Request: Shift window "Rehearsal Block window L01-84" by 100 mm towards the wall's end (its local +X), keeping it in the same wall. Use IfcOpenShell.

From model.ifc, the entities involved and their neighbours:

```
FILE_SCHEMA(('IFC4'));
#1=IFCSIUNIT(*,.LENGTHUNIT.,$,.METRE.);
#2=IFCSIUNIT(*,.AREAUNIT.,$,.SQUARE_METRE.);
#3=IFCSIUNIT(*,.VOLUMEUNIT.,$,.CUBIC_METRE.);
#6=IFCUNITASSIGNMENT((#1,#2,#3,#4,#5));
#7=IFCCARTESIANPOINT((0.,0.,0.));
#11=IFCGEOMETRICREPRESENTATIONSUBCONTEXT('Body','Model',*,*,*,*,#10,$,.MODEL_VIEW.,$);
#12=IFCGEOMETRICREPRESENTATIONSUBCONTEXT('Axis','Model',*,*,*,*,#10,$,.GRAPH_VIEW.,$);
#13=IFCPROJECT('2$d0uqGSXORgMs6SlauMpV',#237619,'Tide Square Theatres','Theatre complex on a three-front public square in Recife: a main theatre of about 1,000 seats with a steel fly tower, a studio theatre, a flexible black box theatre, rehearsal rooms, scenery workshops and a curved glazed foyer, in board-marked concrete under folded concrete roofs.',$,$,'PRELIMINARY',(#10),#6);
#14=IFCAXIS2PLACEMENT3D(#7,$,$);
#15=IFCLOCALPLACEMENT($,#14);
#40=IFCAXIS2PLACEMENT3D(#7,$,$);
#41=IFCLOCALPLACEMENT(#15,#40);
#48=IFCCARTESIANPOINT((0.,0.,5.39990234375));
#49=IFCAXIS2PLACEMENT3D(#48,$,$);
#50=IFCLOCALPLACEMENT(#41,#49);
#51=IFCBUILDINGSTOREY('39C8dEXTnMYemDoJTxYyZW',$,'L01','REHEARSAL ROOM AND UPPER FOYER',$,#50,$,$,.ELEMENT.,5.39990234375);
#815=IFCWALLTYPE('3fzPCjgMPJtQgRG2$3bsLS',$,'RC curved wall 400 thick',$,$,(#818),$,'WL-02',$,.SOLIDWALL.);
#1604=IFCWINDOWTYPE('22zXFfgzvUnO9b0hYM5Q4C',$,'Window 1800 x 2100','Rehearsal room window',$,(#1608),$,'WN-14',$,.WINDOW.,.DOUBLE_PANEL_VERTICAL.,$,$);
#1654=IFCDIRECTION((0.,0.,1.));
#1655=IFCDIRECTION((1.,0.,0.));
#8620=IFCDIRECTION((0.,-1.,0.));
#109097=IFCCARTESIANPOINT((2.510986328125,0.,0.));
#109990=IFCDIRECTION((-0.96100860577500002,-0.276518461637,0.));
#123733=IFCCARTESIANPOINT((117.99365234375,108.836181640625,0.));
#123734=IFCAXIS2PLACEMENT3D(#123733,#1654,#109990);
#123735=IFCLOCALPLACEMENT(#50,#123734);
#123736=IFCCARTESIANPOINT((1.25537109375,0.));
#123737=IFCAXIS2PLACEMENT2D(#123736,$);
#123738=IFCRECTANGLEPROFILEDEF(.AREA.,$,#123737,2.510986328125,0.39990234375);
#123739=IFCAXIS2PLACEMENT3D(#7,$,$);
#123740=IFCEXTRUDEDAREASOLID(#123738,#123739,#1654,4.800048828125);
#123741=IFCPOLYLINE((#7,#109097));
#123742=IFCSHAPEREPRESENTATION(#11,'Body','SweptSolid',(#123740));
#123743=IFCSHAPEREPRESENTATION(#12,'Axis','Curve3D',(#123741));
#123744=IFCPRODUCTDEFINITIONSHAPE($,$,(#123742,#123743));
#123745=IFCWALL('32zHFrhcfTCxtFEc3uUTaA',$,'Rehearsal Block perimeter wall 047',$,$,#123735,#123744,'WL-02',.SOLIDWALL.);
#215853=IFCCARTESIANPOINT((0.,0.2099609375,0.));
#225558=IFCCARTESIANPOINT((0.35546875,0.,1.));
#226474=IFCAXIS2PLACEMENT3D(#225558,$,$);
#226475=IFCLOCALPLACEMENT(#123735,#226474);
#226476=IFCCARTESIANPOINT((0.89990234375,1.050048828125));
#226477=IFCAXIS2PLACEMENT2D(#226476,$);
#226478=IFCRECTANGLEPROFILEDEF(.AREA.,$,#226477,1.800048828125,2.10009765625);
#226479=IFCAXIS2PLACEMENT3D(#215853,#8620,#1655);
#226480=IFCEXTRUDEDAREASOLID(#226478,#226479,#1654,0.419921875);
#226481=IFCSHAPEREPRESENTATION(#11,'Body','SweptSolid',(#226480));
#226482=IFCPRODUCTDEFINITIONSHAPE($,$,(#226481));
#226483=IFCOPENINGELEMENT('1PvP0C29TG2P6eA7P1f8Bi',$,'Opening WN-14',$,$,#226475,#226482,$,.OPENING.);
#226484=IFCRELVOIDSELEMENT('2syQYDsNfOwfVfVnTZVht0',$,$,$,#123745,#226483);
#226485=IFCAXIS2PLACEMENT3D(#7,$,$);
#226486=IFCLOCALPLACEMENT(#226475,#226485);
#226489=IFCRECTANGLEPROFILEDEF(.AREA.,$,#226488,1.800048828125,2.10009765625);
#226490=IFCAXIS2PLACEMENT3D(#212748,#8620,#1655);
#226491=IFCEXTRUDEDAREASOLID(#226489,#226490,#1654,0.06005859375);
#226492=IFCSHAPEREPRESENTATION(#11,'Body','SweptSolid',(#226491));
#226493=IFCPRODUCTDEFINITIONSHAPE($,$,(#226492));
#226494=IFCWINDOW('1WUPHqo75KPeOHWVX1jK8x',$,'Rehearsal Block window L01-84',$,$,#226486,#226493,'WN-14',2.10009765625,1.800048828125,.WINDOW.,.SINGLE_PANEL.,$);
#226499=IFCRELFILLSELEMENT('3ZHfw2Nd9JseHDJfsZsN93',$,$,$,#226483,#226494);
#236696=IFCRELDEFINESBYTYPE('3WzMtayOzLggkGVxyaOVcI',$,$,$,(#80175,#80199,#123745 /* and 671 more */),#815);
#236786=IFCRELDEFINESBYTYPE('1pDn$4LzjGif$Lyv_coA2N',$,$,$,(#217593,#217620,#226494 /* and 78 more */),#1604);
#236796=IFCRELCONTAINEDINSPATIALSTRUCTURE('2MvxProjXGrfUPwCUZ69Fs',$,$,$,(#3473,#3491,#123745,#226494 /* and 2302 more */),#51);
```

```python
import ifcopenshell
import ifcopenshell.api.geometry
import ifcopenshell.util.placement

model = ifcopenshell.open("model.ifc")

window = model.by_guid("1WUPHqo75KPeOHWVX1jK8x")
opening = window.FillsVoids[0].RelatingOpeningElement
wall = opening.VoidsElements[0].RelatingBuildingElement

wall_matrix = ifcopenshell.util.placement.get_local_placement(wall.ObjectPlacement)
shift = wall_matrix[:3, 0] * 0.1
before = ifcopenshell.util.placement.get_local_placement(window.ObjectPlacement)[:3, 3].copy()

# The window is placed relative to its opening, so it follows when the opening moves.
matrix = ifcopenshell.util.placement.get_local_placement(opening.ObjectPlacement)
matrix[:3, 3] += shift
ifcopenshell.api.geometry.edit_object_placement(
    model, product=opening, matrix=matrix, is_si=False, should_transform_children=True
)

after = ifcopenshell.util.placement.get_local_placement(window.ObjectPlacement)[:3, 3]
print("window moved by", (after - before).round(3) + 0.0)

model.write("model_v2.ifc")
```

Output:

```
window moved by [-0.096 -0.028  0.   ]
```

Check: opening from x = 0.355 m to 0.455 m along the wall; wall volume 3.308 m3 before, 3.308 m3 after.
